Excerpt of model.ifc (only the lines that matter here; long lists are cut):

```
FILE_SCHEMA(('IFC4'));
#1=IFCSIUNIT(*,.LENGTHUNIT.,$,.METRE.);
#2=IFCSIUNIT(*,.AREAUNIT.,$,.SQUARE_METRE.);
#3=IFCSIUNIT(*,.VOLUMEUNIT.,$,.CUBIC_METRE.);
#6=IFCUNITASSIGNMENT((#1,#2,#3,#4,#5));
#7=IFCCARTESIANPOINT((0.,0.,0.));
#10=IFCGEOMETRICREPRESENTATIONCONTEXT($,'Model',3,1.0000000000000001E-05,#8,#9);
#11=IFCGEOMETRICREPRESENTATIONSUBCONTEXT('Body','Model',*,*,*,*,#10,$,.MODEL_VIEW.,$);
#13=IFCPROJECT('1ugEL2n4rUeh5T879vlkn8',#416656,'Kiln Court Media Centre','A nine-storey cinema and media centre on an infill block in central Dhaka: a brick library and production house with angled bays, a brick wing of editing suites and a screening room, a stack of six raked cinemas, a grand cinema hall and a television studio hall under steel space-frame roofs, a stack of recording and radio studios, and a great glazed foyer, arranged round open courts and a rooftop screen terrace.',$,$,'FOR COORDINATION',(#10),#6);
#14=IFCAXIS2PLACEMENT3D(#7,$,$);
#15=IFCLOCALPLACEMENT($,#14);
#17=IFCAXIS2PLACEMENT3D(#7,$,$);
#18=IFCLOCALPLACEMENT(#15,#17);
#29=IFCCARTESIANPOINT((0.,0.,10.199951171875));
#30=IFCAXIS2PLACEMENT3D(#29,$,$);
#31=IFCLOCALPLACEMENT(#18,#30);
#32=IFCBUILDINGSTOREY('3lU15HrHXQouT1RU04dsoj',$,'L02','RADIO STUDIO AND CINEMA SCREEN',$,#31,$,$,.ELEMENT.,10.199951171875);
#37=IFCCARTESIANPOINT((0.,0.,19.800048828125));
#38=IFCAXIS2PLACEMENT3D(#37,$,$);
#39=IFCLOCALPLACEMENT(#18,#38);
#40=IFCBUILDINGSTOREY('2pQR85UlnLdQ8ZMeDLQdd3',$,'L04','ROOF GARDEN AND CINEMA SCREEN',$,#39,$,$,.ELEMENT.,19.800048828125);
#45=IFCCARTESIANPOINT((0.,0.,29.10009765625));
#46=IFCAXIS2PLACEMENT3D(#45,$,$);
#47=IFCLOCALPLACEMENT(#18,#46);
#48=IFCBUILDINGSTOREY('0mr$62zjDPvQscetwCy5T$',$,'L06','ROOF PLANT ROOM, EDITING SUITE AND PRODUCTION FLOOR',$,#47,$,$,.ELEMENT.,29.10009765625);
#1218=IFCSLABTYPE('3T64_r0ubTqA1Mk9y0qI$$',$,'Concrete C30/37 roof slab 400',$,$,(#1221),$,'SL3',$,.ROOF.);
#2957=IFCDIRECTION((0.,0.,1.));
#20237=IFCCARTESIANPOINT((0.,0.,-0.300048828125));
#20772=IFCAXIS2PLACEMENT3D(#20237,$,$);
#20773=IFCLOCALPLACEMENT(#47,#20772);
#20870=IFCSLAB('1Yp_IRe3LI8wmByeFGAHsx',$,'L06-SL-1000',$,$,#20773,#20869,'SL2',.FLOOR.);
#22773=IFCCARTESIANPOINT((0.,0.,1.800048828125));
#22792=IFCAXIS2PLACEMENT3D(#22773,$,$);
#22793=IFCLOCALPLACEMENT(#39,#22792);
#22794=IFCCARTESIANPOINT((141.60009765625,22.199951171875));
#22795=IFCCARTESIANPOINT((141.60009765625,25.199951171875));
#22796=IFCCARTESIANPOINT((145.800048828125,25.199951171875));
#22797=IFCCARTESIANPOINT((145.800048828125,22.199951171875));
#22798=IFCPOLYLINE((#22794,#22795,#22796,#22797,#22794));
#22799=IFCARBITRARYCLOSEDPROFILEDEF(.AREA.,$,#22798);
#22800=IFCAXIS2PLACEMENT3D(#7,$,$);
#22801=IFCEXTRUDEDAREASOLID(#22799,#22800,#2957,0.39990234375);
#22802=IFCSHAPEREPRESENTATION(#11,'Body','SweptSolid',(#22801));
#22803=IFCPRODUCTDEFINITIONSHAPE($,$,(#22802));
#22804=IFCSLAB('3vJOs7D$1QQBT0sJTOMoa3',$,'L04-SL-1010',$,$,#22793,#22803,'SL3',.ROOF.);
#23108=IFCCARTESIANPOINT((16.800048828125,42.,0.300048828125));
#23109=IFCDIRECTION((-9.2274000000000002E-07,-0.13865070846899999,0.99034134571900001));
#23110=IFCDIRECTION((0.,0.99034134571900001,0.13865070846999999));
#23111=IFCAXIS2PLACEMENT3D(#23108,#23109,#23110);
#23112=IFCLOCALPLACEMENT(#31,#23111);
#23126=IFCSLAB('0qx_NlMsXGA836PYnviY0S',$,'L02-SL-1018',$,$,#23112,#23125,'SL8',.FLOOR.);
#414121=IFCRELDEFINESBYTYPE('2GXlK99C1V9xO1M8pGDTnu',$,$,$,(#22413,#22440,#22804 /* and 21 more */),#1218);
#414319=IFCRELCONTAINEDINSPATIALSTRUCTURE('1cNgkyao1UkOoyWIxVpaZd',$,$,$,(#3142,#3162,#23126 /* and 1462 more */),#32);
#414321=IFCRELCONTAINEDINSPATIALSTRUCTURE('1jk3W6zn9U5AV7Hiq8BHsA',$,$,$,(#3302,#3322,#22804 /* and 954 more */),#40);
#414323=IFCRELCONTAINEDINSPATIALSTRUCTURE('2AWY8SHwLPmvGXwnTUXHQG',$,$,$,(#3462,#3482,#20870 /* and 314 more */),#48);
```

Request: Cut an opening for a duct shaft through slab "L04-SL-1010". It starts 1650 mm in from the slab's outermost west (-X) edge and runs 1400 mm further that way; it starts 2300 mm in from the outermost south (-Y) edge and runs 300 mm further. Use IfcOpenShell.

```python
import numpy as np
import ifcopenshell
import ifcopenshell.api.feature
import ifcopenshell.api.geometry
import ifcopenshell.api.root
import ifcopenshell.geom
import ifcopenshell.util.placement
import ifcopenshell.util.representation
import ifcopenshell.util.shape
import ifcopenshell.util.unit

model = ifcopenshell.open("model.ifc")
unit_scale = ifcopenshell.util.unit.calculate_unit_scale(model)
settings = ifcopenshell.geom.settings()


def volume(element):
    """Net volume in cubic metres, openings subtracted."""
    shape = ifcopenshell.geom.create_shape(settings, element)
    return ifcopenshell.util.shape.get_volume(shape.geometry)


slab = model.by_guid("3vJOs7D$1QQBT0sJTOMoa3")
before = volume(slab)

# Extent in the slab's own axes, in metres. The edges named are its -X and -Y sides.
slab_shape = ifcopenshell.geom.create_shape(settings, slab)
vertices = ifcopenshell.util.shape.get_vertices(slab_shape.geometry)
x_min, y_min, bottom = vertices.min(axis=0)
top = vertices[:, 2].max()

opening = ifcopenshell.api.root.create_entity(model, ifc_class="IfcOpeningElement", name="Duct shaft opening", predefined_type="OPENING")
context = ifcopenshell.util.representation.get_context(model, "Model", "Body", "MODEL_VIEW")
width, depth = 1.4, 0.3
outline = [(0.0, 0.0), (width, 0.0), (width, depth), (0.0, depth), (0.0, 0.0)]
# Overshoot both faces by 50 mm so the cut is clean.
shape = ifcopenshell.api.geometry.add_slab_representation(
    model, context=context, depth=top - bottom + 0.1, polyline=outline
)
ifcopenshell.api.geometry.assign_representation(model, product=opening, representation=shape)

matrix = ifcopenshell.util.placement.get_local_placement(slab.ObjectPlacement)
matrix[:, 3] = matrix @ np.append(np.array([x_min + 1.65, y_min + 2.3, bottom - 0.05]) / unit_scale, 1.0)
ifcopenshell.api.geometry.edit_object_placement(model, product=opening, matrix=matrix, is_si=False)
ifcopenshell.api.feature.add_feature(model, feature=opening, element=slab)

after = volume(slab)

print(f"slab volume {before:.3f} -> {after:.3f} m3")

model.write("model_updated.ifc")
```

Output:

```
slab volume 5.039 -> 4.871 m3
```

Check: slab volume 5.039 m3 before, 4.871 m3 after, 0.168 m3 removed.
